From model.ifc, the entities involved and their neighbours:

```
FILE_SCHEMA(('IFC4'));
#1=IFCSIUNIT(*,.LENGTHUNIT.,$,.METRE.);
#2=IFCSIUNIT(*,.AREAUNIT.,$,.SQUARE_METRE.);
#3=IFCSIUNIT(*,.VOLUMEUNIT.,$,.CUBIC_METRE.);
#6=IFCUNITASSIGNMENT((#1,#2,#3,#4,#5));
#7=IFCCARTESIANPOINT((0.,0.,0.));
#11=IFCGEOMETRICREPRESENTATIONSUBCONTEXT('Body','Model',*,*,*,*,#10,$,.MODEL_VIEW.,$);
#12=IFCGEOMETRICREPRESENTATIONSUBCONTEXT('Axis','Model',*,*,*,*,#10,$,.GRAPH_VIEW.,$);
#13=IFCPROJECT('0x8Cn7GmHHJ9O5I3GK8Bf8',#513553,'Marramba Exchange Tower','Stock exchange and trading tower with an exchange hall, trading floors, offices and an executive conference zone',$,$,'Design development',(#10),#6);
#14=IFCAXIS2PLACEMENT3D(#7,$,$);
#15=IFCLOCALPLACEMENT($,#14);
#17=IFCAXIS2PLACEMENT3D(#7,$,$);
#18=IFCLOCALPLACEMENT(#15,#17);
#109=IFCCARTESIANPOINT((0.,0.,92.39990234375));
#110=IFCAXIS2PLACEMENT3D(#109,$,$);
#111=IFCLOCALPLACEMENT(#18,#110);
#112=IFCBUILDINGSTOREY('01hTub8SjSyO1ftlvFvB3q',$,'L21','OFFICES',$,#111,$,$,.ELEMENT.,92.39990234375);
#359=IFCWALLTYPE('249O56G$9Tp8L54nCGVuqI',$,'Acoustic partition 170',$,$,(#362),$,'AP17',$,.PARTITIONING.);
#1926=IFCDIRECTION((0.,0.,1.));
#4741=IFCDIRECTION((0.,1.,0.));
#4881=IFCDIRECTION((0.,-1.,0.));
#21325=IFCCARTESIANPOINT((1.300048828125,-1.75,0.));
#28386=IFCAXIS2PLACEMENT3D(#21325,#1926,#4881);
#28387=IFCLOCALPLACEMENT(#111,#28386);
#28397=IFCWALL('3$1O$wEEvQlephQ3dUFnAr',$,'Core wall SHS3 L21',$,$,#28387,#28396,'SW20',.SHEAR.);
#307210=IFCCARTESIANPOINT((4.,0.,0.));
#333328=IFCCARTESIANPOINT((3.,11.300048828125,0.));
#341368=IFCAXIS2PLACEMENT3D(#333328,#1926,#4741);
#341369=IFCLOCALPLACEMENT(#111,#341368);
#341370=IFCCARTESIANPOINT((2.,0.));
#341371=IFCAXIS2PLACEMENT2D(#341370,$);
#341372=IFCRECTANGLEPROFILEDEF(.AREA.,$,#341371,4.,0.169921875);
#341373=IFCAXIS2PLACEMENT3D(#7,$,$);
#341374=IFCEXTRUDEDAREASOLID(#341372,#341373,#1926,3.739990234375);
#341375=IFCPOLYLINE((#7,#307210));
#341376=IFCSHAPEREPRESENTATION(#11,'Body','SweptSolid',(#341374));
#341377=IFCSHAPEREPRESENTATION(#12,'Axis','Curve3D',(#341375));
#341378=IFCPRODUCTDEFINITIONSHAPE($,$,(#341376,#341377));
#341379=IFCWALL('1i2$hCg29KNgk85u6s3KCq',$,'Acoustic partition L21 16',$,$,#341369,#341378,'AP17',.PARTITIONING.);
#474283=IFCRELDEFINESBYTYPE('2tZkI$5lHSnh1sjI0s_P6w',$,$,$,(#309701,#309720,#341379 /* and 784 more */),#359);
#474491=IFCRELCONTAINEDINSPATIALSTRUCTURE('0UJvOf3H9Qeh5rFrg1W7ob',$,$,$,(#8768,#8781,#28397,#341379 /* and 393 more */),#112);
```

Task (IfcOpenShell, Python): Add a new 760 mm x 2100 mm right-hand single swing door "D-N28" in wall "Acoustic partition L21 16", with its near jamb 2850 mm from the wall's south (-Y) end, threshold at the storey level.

```python
import numpy as np
import ifcopenshell
import ifcopenshell.api.feature
import ifcopenshell.api.geometry
import ifcopenshell.api.root
import ifcopenshell.api.spatial
import ifcopenshell.geom
import ifcopenshell.util.element
import ifcopenshell.util.placement
import ifcopenshell.util.representation
import ifcopenshell.util.shape
import ifcopenshell.util.unit

model = ifcopenshell.open("model.ifc")
unit_scale = ifcopenshell.util.unit.calculate_unit_scale(model)
settings = ifcopenshell.geom.settings()


def volume(element):
    """Net volume in cubic metres, openings subtracted."""
    shape = ifcopenshell.geom.create_shape(settings, element)
    return ifcopenshell.util.shape.get_volume(shape.geometry)


wall = model.by_id(341379)
storey = ifcopenshell.util.element.get_container(wall, ifc_class="IfcBuildingStorey")
context = ifcopenshell.util.representation.get_context(model, "Model", "Body", "MODEL_VIEW")
before = volume(wall)

width, height, from_end, sill = 0.76, 2.1, 2.85, 0.0  # metres

# The wall runs along its own X axis, and the end named is its -X end.
wall_shape = ifcopenshell.geom.create_shape(settings, wall)
x, y, z = ifcopenshell.util.shape.get_vertices(wall_shape.geometry).T
start = x.min() + from_end
face, thickness = float(y.min()), float(y.max() - y.min())
wall_matrix = ifcopenshell.util.placement.get_local_placement(wall.ObjectPlacement)
level = ifcopenshell.util.placement.get_local_placement(storey.ObjectPlacement)[2, 3]


def in_wall(x, y):
    """Placement at x, y metres in the wall's axes, at sill height."""
    matrix = wall_matrix.copy()
    matrix[:, 3] = wall_matrix @ np.array([x / unit_scale, y / unit_scale, 0.0, 1.0])
    matrix[2, 3] = level + sill / unit_scale
    return matrix


# Opening: a box that overshoots both wall faces by 50 mm.
opening = ifcopenshell.api.root.create_entity(model, ifc_class="IfcOpeningElement", predefined_type="OPENING")
box = ifcopenshell.api.geometry.add_wall_representation(
    model, context=context, length=width, height=height, thickness=thickness + 0.1
)
ifcopenshell.api.geometry.assign_representation(model, product=opening, representation=box)
ifcopenshell.api.geometry.edit_object_placement(model, product=opening, matrix=in_wall(start, face - 0.05), is_si=False)
ifcopenshell.api.feature.add_feature(model, feature=opening, element=wall)

door = ifcopenshell.api.root.create_entity(model, ifc_class="IfcDoor", name="D-N28", predefined_type="DOOR")
door.OverallWidth, door.OverallHeight = width / unit_scale, height / unit_scale
door.OperationType = "SINGLE_SWING_RIGHT"
body = ifcopenshell.api.geometry.add_door_representation(
    model,
    context=context,
    overall_width=door.OverallWidth,
    overall_height=door.OverallHeight,
    operation_type="SINGLE_SWING_RIGHT",
    lining_properties={"LiningDepth": thickness / unit_scale, "ThresholdDepth": thickness / unit_scale},
)
ifcopenshell.api.geometry.assign_representation(model, product=door, representation=body)
ifcopenshell.api.spatial.assign_container(model, products=[door], relating_structure=storey)
ifcopenshell.api.feature.add_filling(model, opening=opening, element=door)

# The lining spans the wall, so the door starts at the wall face.
ifcopenshell.api.geometry.edit_object_placement(model, product=door, matrix=in_wall(start, face), is_si=False)

after = volume(wall)

print(f"wall volume {before:.3f} -> {after:.3f} m3")

model.write("model-out.ifc")
```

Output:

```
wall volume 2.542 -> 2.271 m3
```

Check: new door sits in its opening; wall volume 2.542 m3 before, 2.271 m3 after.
